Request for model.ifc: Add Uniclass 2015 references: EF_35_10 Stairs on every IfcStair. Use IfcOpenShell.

First a look at what the model holds.

```python
import ifcopenshell

model = ifcopenshell.open("model.ifc")
print(model.schema)
print("classifications:", [c.Name for c in model.by_type("IfcClassification")])
for ifc_class in ("IfcDoor", "IfcRoof", "IfcStair", "IfcWall", "IfcWindow"):
    print(ifc_class, len(model.by_type(ifc_class)))
```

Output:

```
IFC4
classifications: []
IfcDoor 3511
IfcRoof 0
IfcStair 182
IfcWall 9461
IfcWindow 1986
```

```python
import ifcopenshell
import ifcopenshell.api.classification

model = ifcopenshell.open("model.ifc")

system = ifcopenshell.api.classification.add_classification(model, classification="Uniclass 2015")

codes = {
    "IfcStair": ("EF_35_10", "Stairs"),
}
for ifc_class, (code, name) in codes.items():
    products = model.by_type(ifc_class)
    ifcopenshell.api.classification.add_reference(
        model, products=products, classification=system, identification=code, name=name
    )
    print(code, len(products))

model.write("model-out.ifc")
```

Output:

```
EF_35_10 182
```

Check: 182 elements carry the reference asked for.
